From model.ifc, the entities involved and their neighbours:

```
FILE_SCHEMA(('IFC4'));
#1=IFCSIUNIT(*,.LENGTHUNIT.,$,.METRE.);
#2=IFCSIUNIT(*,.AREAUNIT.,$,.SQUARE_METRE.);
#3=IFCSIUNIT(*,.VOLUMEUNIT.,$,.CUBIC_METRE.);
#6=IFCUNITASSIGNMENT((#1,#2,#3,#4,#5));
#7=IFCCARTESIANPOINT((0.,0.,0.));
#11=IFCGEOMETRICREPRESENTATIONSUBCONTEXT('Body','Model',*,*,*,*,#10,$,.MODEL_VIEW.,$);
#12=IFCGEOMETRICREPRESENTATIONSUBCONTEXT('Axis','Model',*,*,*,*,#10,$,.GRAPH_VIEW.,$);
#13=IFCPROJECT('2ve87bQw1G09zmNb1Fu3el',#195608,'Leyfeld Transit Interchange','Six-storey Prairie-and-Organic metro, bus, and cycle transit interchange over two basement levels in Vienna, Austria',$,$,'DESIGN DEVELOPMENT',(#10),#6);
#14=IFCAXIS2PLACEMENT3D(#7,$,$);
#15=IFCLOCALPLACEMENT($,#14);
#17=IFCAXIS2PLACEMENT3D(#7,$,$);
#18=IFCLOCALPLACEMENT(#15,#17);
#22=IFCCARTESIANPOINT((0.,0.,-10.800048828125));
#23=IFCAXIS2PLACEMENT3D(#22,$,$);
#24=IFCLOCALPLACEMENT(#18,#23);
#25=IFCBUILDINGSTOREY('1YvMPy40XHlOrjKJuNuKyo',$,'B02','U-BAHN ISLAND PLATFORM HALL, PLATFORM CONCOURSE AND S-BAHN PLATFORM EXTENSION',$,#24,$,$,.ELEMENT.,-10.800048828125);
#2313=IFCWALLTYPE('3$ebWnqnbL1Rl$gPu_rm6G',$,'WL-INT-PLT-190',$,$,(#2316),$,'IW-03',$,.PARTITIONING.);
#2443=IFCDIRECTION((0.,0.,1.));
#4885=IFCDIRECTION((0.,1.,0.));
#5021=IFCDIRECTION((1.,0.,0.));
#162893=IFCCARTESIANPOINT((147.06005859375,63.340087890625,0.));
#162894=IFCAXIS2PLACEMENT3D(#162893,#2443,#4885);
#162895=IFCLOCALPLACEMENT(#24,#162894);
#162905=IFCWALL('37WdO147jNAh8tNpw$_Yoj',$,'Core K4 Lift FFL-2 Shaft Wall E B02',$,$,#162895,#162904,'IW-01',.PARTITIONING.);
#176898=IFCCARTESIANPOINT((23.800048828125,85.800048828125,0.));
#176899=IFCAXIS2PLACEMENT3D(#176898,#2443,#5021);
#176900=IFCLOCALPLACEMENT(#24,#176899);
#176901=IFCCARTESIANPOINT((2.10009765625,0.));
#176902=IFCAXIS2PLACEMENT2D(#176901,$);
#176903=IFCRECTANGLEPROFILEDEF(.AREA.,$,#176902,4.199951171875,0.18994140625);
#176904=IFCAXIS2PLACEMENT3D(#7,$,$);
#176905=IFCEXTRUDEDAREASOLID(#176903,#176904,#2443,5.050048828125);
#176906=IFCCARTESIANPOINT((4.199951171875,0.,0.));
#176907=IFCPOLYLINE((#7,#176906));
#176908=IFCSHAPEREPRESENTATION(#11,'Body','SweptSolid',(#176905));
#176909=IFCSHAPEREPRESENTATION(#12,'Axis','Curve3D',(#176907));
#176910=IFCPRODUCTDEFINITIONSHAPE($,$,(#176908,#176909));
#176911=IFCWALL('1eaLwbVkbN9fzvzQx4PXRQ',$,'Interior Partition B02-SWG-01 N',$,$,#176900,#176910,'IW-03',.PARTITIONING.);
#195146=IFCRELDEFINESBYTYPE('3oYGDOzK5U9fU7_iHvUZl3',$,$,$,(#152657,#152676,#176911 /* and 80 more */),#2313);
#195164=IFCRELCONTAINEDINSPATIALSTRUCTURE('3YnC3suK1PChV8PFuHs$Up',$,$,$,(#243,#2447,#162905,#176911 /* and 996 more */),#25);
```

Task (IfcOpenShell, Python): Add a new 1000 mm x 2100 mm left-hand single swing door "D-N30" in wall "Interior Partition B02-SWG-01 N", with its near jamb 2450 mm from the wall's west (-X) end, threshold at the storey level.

```python
import numpy as np
import ifcopenshell
import ifcopenshell.api.feature
import ifcopenshell.api.geometry
import ifcopenshell.api.root
import ifcopenshell.api.spatial
import ifcopenshell.geom
import ifcopenshell.util.element
import ifcopenshell.util.placement
import ifcopenshell.util.representation
import ifcopenshell.util.shape
import ifcopenshell.util.unit

model = ifcopenshell.open("model.ifc")
unit_scale = ifcopenshell.util.unit.calculate_unit_scale(model)
settings = ifcopenshell.geom.settings()


def volume(element):
    """Net volume in cubic metres, openings subtracted."""
    shape = ifcopenshell.geom.create_shape(settings, element)
    return ifcopenshell.util.shape.get_volume(shape.geometry)


wall = model.by_guid("1eaLwbVkbN9fzvzQx4PXRQ")
storey = ifcopenshell.util.element.get_container(wall, ifc_class="IfcBuildingStorey")
context = ifcopenshell.util.representation.get_context(model, "Model", "Body", "MODEL_VIEW")
before = volume(wall)

width, height, from_end, sill = 1, 2.1, 2.45, 0.0  # metres

# The wall runs along its own X axis, and the end named is its -X end.
wall_shape = ifcopenshell.geom.create_shape(settings, wall)
x, y, z = ifcopenshell.util.shape.get_vertices(wall_shape.geometry).T
start = x.min() + from_end
face, thickness = float(y.min()), float(y.max() - y.min())
wall_matrix = ifcopenshell.util.placement.get_local_placement(wall.ObjectPlacement)
level = ifcopenshell.util.placement.get_local_placement(storey.ObjectPlacement)[2, 3]


def in_wall(x, y):
    """Placement at x, y metres in the wall's axes, at sill height."""
    matrix = wall_matrix.copy()
    matrix[:, 3] = wall_matrix @ np.array([x / unit_scale, y / unit_scale, 0.0, 1.0])
    matrix[2, 3] = level + sill / unit_scale
    return matrix


# Opening: a box that overshoots both wall faces by 50 mm.
opening = ifcopenshell.api.root.create_entity(model, ifc_class="IfcOpeningElement", predefined_type="OPENING")
box = ifcopenshell.api.geometry.add_wall_representation(
    model, context=context, length=width, height=height, thickness=thickness + 0.1
)
ifcopenshell.api.geometry.assign_representation(model, product=opening, representation=box)
ifcopenshell.api.geometry.edit_object_placement(model, product=opening, matrix=in_wall(start, face - 0.05), is_si=False)
ifcopenshell.api.feature.add_feature(model, feature=opening, element=wall)

door = ifcopenshell.api.root.create_entity(model, ifc_class="IfcDoor", name="D-N30", predefined_type="DOOR")
door.OverallWidth, door.OverallHeight = width / unit_scale, height / unit_scale
door.OperationType = "SINGLE_SWING_LEFT"
body = ifcopenshell.api.geometry.add_door_representation(
    model,
    context=context,
    overall_width=door.OverallWidth,
    overall_height=door.OverallHeight,
    operation_type="SINGLE_SWING_LEFT",
    lining_properties={"LiningDepth": thickness / unit_scale, "ThresholdDepth": thickness / unit_scale},
)
ifcopenshell.api.geometry.assign_representation(model, product=door, representation=body)
ifcopenshell.api.spatial.assign_container(model, products=[door], relating_structure=storey)
ifcopenshell.api.feature.add_filling(model, opening=opening, element=door)

# The lining spans the wall, so the door starts at the wall face.
ifcopenshell.api.geometry.edit_object_placement(model, product=door, matrix=in_wall(start, face), is_si=False)

after = volume(wall)

print(f"wall volume {before:.3f} -> {after:.3f} m3")

model.write("model-out.ifc")
```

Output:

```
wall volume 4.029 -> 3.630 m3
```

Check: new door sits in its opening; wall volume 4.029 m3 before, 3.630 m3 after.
